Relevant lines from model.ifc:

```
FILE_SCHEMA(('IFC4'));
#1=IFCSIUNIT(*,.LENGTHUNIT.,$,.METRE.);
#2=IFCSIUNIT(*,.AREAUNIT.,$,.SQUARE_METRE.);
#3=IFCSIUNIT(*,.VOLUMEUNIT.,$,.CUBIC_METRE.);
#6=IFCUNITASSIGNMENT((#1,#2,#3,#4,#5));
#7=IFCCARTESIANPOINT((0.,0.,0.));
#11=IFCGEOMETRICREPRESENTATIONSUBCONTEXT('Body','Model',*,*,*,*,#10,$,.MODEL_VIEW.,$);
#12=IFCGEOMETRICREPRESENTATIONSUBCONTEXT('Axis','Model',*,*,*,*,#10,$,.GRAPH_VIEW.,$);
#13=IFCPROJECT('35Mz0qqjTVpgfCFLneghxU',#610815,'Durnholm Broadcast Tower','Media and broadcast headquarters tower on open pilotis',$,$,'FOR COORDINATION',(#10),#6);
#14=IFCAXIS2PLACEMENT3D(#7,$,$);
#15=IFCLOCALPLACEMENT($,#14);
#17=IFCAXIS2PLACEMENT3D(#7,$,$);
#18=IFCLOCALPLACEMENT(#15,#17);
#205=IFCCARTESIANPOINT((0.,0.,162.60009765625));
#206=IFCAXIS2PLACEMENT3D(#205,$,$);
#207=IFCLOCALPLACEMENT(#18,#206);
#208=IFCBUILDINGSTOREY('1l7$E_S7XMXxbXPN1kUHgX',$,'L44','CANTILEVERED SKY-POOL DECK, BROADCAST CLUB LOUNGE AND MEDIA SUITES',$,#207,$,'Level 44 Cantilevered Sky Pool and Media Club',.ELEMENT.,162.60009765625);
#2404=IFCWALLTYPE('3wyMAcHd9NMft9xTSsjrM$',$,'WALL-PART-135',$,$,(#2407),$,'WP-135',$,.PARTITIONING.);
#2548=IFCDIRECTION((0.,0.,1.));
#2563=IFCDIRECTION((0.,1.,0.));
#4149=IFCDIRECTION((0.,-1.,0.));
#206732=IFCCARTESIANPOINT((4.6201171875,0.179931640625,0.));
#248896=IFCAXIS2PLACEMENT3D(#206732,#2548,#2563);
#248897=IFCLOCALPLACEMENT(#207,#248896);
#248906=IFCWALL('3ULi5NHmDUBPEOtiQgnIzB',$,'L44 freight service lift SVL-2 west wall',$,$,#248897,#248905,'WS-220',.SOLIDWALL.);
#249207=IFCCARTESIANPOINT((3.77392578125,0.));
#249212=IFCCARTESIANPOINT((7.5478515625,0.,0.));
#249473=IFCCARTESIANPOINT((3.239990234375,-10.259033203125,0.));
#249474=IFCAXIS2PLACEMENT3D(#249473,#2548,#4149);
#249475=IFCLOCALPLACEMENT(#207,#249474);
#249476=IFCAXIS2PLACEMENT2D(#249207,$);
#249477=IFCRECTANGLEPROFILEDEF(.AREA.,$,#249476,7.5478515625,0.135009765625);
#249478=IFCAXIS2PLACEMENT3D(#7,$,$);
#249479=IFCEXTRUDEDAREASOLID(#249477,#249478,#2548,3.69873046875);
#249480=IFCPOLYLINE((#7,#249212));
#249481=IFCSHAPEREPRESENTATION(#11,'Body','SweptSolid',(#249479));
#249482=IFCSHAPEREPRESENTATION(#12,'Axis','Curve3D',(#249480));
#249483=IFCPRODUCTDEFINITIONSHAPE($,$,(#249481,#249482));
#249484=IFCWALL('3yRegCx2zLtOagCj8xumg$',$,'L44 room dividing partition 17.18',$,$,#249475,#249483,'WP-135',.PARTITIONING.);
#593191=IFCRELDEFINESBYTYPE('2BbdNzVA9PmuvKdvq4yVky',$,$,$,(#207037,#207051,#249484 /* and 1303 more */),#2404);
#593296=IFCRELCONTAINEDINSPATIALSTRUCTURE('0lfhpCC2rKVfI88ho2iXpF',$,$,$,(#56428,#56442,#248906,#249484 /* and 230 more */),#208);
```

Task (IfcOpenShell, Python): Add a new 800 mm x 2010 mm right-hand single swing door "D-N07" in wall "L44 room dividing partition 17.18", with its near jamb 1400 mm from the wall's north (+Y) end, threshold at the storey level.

```python
import numpy as np
import ifcopenshell
import ifcopenshell.api.feature
import ifcopenshell.api.geometry
import ifcopenshell.api.root
import ifcopenshell.api.spatial
import ifcopenshell.geom
import ifcopenshell.util.element
import ifcopenshell.util.placement
import ifcopenshell.util.representation
import ifcopenshell.util.shape
import ifcopenshell.util.unit

model = ifcopenshell.open("model.ifc")
unit_scale = ifcopenshell.util.unit.calculate_unit_scale(model)
settings = ifcopenshell.geom.settings()


def volume(element):
    """Net volume in cubic metres, openings subtracted."""
    shape = ifcopenshell.geom.create_shape(settings, element)
    return ifcopenshell.util.shape.get_volume(shape.geometry)


wall = model.by_guid("3yRegCx2zLtOagCj8xumg$")
storey = ifcopenshell.util.element.get_container(wall, ifc_class="IfcBuildingStorey")
context = ifcopenshell.util.representation.get_context(model, "Model", "Body", "MODEL_VIEW")
before = volume(wall)

width, height, from_end, sill = 0.8, 2.01, 1.4, 0.0  # metres

# The wall runs along its own X axis, and the end named is its -X end.
wall_shape = ifcopenshell.geom.create_shape(settings, wall)
x, y, z = ifcopenshell.util.shape.get_vertices(wall_shape.geometry).T
start = x.min() + from_end
face, thickness = float(y.min()), float(y.max() - y.min())
wall_matrix = ifcopenshell.util.placement.get_local_placement(wall.ObjectPlacement)
level = ifcopenshell.util.placement.get_local_placement(storey.ObjectPlacement)[2, 3]


def in_wall(x, y):
    """Placement at x, y metres in the wall's axes, at sill height."""
    matrix = wall_matrix.copy()
    matrix[:, 3] = wall_matrix @ np.array([x / unit_scale, y / unit_scale, 0.0, 1.0])
    matrix[2, 3] = level + sill / unit_scale
    return matrix


# Opening: a box that overshoots both wall faces by 50 mm.
opening = ifcopenshell.api.root.create_entity(model, ifc_class="IfcOpeningElement", predefined_type="OPENING")
box = ifcopenshell.api.geometry.add_wall_representation(
    model, context=context, length=width, height=height, thickness=thickness + 0.1
)
ifcopenshell.api.geometry.assign_representation(model, product=opening, representation=box)
ifcopenshell.api.geometry.edit_object_placement(model, product=opening, matrix=in_wall(start, face - 0.05), is_si=False)
ifcopenshell.api.feature.add_feature(model, feature=opening, element=wall)

door = ifcopenshell.api.root.create_entity(model, ifc_class="IfcDoor", name="D-N07", predefined_type="DOOR")
door.OverallWidth, door.OverallHeight = width / unit_scale, height / unit_scale
door.OperationType = "SINGLE_SWING_RIGHT"
body = ifcopenshell.api.geometry.add_door_representation(
    model,
    context=context,
    overall_width=door.OverallWidth,
    overall_height=door.OverallHeight,
    operation_type="SINGLE_SWING_RIGHT",
    lining_properties={"LiningDepth": thickness / unit_scale, "ThresholdDepth": thickness / unit_scale},
)
ifcopenshell.api.geometry.assign_representation(model, product=door, representation=body)
ifcopenshell.api.spatial.assign_container(model, products=[door], relating_structure=storey)
ifcopenshell.api.feature.add_filling(model, opening=opening, element=door)

# The lining spans the wall, so the door starts at the wall face.
ifcopenshell.api.geometry.edit_object_placement(model, product=door, matrix=in_wall(start, face), is_si=False)

after = volume(wall)

print(f"wall volume {before:.3f} -> {after:.3f} m3")

model.write("model_updated.ifc")
```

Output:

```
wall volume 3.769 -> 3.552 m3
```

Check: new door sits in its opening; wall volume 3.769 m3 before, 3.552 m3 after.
